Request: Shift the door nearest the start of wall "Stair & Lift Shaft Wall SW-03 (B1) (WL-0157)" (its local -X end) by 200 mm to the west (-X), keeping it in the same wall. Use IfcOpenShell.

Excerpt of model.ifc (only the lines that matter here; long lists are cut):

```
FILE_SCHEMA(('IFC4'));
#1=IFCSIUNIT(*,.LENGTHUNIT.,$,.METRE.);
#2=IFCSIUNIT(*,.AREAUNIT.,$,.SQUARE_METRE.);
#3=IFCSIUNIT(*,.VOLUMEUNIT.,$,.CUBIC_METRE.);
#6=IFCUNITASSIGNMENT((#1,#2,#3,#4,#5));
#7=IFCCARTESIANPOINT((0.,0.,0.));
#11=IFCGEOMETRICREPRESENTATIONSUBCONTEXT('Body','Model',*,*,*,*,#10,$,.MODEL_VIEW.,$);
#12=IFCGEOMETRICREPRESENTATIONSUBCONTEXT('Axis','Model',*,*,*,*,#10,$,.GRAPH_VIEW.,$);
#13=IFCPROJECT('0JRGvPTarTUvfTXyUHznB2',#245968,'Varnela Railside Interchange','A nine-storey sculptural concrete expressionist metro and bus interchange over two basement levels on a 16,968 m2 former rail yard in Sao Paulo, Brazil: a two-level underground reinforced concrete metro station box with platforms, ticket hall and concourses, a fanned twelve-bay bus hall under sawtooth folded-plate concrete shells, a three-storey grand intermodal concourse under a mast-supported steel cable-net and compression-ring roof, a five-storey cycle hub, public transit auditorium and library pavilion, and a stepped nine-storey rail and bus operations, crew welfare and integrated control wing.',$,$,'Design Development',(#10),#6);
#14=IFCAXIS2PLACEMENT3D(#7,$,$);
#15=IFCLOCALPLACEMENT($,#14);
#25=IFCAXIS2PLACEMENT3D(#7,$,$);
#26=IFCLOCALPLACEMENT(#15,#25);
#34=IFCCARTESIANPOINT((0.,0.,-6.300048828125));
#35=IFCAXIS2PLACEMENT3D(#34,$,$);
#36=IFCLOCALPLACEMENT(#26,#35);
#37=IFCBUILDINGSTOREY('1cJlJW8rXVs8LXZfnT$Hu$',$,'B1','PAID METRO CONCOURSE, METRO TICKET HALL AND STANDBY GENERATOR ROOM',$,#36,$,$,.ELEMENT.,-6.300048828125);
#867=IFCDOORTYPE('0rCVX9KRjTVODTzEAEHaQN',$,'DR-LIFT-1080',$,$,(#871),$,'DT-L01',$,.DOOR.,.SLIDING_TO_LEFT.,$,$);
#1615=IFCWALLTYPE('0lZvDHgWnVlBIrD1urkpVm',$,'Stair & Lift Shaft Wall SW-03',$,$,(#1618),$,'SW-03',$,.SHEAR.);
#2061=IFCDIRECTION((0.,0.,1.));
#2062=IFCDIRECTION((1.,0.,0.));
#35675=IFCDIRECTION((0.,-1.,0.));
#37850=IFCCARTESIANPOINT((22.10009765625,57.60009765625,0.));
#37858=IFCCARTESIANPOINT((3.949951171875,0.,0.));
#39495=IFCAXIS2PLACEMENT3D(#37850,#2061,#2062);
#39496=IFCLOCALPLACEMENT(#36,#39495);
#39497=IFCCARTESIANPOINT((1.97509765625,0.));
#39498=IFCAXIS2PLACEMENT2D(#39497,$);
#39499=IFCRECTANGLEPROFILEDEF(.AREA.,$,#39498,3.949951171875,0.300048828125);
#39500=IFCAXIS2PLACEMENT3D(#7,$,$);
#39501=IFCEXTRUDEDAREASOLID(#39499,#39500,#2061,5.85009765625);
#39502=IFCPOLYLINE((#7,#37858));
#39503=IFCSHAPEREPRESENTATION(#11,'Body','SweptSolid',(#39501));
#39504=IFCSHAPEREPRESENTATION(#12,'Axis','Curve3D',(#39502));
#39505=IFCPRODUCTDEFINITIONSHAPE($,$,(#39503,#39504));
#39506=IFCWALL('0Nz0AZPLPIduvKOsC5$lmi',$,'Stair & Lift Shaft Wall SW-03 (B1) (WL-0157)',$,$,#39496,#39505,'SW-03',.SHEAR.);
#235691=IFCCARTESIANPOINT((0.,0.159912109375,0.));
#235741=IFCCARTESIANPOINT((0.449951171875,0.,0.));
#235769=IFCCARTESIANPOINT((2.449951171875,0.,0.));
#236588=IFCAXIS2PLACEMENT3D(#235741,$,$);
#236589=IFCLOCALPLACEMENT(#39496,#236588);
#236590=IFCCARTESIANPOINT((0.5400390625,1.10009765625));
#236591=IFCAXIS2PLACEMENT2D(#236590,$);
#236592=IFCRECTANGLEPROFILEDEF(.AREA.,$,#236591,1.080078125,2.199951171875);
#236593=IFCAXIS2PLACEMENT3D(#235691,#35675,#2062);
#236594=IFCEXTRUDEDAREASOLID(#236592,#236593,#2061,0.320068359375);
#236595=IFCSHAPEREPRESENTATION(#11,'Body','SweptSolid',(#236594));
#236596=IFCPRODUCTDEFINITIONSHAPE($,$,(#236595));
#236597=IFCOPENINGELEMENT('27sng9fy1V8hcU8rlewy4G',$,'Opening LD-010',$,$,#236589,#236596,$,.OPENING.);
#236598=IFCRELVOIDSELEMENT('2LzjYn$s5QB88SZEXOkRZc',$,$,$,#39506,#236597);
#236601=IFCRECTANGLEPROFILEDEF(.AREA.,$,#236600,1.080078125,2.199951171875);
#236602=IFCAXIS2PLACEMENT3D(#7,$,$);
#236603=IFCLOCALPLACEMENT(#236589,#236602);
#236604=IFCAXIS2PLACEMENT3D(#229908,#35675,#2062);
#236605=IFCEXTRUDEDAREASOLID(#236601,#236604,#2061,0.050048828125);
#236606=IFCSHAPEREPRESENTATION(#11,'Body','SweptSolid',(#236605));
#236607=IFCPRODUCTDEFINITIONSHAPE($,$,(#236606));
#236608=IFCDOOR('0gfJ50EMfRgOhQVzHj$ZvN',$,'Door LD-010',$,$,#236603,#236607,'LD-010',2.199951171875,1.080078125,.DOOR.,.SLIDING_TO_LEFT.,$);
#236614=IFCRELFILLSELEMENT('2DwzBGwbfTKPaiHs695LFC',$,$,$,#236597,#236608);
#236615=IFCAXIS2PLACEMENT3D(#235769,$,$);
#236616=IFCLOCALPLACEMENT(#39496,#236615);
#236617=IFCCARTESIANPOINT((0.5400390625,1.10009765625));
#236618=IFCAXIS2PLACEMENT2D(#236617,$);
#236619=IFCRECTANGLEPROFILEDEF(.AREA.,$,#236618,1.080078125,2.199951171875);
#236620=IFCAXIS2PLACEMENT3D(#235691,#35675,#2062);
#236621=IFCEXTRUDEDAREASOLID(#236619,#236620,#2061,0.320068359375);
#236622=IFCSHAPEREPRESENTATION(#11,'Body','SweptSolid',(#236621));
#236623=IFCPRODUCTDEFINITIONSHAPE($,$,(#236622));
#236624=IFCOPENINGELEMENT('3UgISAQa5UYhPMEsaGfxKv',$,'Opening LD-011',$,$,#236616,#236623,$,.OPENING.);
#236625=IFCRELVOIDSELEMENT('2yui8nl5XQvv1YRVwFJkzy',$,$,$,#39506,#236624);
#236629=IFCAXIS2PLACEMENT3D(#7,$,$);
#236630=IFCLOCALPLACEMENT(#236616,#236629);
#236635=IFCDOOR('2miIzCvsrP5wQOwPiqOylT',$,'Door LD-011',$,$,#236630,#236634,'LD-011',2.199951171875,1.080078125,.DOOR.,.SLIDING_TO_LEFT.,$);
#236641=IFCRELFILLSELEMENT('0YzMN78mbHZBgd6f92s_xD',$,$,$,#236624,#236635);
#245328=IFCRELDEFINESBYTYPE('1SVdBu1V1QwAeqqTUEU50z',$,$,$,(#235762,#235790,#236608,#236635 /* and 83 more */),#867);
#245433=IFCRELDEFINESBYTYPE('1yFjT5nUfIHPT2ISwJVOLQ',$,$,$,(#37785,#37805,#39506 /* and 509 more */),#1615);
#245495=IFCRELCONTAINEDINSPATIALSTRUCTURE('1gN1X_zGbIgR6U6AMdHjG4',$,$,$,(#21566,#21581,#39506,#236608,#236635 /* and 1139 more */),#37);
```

```python
import ifcopenshell
import ifcopenshell.api.geometry
import ifcopenshell.util.placement
import ifcopenshell.util.unit

model = ifcopenshell.open("model.ifc")
unit_scale = ifcopenshell.util.unit.calculate_unit_scale(model)

door = model.by_guid("0gfJ50EMfRgOhQVzHj$ZvN")
opening = door.FillsVoids[0].RelatingOpeningElement
wall = opening.VoidsElements[0].RelatingBuildingElement

wall_matrix = ifcopenshell.util.placement.get_local_placement(wall.ObjectPlacement)
shift = wall_matrix[:3, 0] * -0.2 / unit_scale
before = ifcopenshell.util.placement.get_local_placement(door.ObjectPlacement)[:3, 3].copy()

# The door is placed relative to its opening, so it follows when the opening moves.
matrix = ifcopenshell.util.placement.get_local_placement(opening.ObjectPlacement)
matrix[:3, 3] += shift
ifcopenshell.api.geometry.edit_object_placement(
    model, product=opening, matrix=matrix, is_si=False, should_transform_children=True
)

after = ifcopenshell.util.placement.get_local_placement(door.ObjectPlacement)[:3, 3]
print("door moved by", (after - before).round(3) + 0.0)

model.write("model_v2.ifc")
```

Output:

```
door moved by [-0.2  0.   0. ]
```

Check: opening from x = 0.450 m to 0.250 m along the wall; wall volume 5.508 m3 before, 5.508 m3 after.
